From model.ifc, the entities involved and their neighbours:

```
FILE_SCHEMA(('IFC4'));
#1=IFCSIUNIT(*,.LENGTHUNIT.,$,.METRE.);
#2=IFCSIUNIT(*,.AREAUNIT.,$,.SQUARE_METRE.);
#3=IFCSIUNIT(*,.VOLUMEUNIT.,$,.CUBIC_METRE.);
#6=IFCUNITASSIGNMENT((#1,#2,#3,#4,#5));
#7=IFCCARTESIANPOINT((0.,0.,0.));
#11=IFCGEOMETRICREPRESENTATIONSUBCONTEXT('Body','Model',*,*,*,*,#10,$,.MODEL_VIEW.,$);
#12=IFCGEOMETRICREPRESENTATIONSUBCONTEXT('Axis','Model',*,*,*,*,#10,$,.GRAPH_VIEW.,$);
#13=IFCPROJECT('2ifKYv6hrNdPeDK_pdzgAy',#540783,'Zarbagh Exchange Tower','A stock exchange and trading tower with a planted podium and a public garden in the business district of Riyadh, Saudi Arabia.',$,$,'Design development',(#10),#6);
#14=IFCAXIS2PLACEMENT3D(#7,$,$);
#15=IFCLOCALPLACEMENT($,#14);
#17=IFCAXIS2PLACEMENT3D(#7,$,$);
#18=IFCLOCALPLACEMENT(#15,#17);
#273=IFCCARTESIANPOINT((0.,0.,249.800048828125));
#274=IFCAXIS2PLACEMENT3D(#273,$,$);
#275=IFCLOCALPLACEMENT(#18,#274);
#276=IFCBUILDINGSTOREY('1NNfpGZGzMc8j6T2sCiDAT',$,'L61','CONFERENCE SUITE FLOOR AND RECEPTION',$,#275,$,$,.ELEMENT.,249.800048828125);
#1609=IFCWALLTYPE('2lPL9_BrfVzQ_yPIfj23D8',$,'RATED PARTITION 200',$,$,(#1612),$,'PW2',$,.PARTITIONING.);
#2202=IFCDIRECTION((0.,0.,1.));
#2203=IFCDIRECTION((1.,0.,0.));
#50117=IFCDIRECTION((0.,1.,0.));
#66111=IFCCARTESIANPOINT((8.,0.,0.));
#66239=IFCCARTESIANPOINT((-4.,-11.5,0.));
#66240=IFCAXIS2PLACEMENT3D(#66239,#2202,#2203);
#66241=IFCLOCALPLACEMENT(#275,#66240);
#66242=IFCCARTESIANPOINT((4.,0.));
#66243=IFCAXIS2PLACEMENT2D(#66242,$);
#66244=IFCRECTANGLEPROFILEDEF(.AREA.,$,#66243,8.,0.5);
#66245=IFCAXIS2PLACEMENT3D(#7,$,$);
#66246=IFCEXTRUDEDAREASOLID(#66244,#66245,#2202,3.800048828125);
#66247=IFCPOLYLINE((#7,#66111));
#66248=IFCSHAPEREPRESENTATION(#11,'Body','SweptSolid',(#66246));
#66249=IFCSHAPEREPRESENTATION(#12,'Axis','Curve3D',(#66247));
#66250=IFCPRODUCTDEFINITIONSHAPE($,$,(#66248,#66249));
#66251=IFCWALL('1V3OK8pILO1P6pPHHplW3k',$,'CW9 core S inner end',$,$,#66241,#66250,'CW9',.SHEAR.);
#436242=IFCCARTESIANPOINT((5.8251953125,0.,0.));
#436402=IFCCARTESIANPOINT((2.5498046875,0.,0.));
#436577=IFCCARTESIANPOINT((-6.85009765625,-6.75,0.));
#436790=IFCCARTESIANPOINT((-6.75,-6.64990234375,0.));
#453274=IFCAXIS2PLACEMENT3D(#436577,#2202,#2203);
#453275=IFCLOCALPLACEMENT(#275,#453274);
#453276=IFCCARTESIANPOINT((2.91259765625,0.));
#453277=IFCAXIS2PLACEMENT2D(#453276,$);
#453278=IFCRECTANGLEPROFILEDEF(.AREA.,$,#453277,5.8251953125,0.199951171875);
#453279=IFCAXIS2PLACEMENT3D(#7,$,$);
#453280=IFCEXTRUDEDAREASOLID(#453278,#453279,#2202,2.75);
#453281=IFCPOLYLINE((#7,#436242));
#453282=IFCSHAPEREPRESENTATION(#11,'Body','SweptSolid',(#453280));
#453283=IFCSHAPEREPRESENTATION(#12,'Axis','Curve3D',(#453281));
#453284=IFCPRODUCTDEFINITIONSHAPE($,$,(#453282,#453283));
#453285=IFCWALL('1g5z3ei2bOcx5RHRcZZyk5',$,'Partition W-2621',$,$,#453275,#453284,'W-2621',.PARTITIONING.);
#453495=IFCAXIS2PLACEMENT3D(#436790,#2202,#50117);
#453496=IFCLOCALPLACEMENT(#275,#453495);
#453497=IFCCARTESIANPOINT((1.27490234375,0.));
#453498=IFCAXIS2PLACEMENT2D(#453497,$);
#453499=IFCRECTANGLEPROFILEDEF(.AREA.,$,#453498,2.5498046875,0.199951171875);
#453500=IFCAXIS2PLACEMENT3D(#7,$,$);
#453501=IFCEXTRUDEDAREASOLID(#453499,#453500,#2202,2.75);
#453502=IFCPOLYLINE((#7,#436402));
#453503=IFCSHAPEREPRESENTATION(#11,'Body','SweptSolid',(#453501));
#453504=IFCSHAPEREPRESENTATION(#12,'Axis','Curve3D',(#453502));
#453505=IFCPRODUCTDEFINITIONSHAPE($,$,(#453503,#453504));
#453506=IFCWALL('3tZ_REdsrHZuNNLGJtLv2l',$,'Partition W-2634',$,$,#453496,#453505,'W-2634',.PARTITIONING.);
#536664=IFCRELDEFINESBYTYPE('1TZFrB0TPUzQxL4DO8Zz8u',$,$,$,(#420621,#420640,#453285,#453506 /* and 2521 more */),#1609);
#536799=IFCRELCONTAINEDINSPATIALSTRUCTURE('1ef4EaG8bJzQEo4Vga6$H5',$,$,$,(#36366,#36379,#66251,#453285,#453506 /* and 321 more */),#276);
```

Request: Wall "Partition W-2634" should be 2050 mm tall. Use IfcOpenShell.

```python
import ifcopenshell
import ifcopenshell.geom
import ifcopenshell.util.representation
import ifcopenshell.util.shape

model = ifcopenshell.open("model.ifc")
settings = ifcopenshell.geom.settings()


def volume(element):
    """Net volume in cubic metres, openings subtracted."""
    shape = ifcopenshell.geom.create_shape(settings, element)
    return ifcopenshell.util.shape.get_volume(shape.geometry)


wall = model.by_guid("3tZ_REdsrHZuNNLGJtLv2l")
before = volume(wall)

body = ifcopenshell.util.representation.get_representation(wall, "Model", "Body")
solid = body.Items[0]
old_height = solid.Depth
solid.Depth = 2.05
after = volume(wall)

print(f"height {old_height:g} -> {solid.Depth:g}, volume {before:.3f} -> {after:.3f} m3")

model.write("model_rev.ifc")
```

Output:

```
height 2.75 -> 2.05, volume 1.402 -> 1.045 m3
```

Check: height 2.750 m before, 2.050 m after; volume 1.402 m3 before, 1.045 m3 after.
